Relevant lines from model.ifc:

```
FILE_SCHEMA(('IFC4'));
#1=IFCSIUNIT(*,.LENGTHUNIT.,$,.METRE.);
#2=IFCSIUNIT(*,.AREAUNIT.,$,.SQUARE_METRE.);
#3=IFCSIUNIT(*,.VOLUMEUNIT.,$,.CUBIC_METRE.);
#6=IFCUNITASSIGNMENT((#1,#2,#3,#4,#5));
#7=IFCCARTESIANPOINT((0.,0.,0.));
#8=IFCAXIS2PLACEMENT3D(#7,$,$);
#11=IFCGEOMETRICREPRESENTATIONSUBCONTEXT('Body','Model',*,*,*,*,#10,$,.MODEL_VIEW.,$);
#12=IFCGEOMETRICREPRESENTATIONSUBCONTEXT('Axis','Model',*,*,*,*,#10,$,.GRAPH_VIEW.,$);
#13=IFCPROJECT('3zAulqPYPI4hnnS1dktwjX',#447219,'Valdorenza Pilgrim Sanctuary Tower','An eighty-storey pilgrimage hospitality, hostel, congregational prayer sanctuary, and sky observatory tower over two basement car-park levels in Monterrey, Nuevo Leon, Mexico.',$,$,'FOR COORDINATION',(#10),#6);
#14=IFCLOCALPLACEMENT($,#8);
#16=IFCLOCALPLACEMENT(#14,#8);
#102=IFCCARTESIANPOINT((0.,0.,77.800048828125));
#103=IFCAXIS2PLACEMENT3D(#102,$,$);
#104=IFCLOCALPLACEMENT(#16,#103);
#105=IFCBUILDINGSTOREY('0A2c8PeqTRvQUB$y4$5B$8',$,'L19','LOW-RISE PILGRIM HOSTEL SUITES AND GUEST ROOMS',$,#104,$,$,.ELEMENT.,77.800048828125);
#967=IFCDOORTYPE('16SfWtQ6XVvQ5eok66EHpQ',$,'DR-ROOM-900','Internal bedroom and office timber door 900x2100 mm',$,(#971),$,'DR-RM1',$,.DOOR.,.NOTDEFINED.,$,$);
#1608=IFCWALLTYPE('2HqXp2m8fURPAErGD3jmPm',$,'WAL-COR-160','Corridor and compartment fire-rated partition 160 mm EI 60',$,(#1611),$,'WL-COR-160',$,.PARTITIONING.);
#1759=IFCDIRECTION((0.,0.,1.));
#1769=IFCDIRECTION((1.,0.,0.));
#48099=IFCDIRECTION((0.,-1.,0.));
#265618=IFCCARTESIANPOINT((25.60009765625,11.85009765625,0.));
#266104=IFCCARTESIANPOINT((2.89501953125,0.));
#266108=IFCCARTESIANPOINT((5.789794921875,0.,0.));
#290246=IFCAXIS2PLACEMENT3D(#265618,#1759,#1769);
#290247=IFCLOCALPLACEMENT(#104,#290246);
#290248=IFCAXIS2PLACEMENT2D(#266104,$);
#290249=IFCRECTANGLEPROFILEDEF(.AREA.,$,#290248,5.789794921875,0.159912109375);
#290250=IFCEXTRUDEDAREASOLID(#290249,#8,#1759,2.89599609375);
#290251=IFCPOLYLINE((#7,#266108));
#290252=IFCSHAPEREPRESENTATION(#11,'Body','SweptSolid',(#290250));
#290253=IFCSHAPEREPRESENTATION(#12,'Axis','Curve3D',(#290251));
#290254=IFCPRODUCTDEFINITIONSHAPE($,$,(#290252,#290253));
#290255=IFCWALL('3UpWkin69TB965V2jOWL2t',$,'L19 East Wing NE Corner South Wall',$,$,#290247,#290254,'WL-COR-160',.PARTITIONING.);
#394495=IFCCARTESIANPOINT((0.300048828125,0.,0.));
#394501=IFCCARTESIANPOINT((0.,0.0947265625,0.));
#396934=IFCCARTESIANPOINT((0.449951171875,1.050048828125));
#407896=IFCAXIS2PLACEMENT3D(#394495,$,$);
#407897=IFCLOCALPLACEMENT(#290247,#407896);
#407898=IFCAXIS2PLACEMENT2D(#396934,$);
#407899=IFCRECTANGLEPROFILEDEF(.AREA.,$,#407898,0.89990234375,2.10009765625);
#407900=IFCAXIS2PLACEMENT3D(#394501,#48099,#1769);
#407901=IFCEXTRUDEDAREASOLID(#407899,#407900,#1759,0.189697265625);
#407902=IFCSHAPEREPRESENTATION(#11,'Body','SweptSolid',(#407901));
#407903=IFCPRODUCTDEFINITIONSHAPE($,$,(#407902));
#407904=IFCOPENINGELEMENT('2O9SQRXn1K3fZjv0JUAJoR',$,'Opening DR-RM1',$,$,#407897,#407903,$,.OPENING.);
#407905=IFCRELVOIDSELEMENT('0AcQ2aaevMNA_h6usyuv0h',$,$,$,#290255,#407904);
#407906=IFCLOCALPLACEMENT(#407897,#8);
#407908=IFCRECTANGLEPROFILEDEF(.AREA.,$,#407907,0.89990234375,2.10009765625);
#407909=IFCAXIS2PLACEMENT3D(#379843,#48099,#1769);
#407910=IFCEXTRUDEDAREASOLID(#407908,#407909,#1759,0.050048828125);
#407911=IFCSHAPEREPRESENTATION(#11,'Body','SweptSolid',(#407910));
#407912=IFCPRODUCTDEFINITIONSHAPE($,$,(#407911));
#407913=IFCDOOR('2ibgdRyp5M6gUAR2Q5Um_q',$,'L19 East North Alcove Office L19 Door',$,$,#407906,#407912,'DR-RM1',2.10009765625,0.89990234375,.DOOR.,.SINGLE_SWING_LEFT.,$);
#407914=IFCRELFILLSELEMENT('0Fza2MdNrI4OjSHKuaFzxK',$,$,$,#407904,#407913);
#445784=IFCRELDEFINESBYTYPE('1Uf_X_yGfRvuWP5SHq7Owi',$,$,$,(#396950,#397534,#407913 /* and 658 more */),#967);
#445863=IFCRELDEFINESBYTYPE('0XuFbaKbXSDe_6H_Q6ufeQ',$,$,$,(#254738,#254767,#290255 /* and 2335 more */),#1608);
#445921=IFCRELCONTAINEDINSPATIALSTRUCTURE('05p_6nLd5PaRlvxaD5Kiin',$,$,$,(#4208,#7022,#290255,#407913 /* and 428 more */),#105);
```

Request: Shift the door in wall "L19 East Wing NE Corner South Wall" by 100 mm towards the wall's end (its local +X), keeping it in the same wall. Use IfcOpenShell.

```python
import ifcopenshell
import ifcopenshell.api.geometry
import ifcopenshell.util.placement

model = ifcopenshell.open("model.ifc")

door = model.by_guid("2ibgdRyp5M6gUAR2Q5Um_q")
opening = door.FillsVoids[0].RelatingOpeningElement
wall = opening.VoidsElements[0].RelatingBuildingElement

wall_matrix = ifcopenshell.util.placement.get_local_placement(wall.ObjectPlacement)
shift = wall_matrix[:3, 0] * 0.1
before = ifcopenshell.util.placement.get_local_placement(door.ObjectPlacement)[:3, 3].copy()

# The door is placed relative to its opening, so it follows when the opening moves.
matrix = ifcopenshell.util.placement.get_local_placement(opening.ObjectPlacement)
matrix[:3, 3] += shift
ifcopenshell.api.geometry.edit_object_placement(
    model, product=opening, matrix=matrix, is_si=False, should_transform_children=True
)

after = ifcopenshell.util.placement.get_local_placement(door.ObjectPlacement)[:3, 3]
print("door moved by", (after - before).round(3) + 0.0)

model.write("model-out.ifc")
```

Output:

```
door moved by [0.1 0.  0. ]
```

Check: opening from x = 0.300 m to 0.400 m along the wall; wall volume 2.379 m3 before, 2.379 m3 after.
